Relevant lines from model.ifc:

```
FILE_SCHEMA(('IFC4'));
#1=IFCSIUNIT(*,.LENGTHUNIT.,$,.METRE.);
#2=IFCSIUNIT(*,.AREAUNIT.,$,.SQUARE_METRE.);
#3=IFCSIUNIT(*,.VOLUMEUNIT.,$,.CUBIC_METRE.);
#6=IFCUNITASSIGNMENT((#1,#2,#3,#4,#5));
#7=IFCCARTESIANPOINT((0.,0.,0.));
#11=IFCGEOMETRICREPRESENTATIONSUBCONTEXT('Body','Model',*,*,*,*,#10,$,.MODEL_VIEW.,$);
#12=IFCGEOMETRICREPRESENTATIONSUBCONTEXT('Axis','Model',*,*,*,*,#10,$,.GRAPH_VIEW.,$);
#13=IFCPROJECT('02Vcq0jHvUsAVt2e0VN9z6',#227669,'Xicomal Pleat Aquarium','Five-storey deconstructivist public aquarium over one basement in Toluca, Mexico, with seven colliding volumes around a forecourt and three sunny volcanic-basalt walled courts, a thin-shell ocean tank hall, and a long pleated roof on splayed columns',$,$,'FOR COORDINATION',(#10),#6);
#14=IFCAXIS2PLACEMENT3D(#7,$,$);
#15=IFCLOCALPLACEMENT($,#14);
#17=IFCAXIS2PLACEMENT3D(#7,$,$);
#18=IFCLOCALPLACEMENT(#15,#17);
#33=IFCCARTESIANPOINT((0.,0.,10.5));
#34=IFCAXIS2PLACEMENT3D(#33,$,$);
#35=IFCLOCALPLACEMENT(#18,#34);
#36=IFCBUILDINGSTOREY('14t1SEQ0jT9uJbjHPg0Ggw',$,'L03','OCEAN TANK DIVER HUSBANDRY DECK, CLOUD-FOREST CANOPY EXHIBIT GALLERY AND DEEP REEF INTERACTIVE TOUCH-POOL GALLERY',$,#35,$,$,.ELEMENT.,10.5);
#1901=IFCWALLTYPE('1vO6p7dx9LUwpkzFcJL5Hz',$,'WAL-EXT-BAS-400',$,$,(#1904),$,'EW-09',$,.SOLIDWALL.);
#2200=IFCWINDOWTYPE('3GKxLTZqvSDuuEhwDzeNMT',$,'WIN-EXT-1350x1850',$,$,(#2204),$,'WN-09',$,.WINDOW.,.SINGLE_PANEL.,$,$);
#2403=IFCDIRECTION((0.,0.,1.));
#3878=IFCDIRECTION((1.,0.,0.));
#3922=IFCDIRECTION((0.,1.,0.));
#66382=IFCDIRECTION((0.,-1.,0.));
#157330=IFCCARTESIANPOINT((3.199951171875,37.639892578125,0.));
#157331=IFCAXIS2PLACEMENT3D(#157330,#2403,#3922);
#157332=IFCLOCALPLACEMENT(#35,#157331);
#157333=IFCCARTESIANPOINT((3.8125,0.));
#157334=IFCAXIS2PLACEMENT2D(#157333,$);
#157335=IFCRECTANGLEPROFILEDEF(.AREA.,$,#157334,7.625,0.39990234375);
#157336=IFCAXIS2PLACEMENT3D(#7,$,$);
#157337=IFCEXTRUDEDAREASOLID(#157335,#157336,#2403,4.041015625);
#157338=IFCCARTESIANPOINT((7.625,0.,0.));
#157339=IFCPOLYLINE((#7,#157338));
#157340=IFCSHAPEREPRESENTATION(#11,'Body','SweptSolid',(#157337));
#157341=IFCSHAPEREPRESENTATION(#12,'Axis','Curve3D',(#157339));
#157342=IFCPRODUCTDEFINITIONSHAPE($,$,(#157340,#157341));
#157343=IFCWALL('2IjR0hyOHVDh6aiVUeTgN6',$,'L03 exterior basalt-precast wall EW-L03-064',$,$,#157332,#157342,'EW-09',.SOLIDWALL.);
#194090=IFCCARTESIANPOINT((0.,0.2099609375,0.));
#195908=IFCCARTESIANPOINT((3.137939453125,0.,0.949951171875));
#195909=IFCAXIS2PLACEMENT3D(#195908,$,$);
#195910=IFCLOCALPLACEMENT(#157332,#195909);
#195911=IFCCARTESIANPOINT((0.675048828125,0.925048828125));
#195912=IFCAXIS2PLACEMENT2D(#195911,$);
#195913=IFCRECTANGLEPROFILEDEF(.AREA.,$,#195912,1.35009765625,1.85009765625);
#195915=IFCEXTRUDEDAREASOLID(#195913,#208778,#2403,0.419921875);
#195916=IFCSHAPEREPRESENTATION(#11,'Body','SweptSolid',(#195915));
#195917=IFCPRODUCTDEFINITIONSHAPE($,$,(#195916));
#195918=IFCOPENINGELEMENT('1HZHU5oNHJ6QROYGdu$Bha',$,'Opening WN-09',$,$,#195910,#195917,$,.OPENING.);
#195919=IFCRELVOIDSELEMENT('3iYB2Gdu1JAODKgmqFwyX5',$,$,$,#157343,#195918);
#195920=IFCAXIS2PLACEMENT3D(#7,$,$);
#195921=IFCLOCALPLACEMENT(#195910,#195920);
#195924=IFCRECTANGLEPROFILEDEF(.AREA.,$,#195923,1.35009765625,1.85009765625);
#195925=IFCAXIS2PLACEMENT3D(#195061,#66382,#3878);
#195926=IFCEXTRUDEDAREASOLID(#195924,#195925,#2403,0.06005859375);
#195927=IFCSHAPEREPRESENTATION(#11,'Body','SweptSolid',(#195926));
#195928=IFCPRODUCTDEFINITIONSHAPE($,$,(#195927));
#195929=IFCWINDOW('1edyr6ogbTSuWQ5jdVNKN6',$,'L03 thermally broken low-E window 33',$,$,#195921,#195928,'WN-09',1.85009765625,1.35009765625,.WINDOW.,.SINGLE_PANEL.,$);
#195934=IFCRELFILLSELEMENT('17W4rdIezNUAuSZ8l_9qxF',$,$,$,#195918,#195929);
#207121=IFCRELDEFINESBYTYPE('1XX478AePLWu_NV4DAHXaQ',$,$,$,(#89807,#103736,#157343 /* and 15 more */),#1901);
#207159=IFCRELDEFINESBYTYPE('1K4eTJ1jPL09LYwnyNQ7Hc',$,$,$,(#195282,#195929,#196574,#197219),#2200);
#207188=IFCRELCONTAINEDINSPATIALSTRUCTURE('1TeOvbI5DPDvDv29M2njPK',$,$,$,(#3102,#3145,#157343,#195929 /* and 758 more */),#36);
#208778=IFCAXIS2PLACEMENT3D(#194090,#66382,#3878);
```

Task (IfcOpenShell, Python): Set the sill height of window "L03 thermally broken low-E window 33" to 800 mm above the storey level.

```python
import numpy as np
import ifcopenshell
import ifcopenshell.api.geometry
import ifcopenshell.geom
import ifcopenshell.util.element
import ifcopenshell.util.placement
import ifcopenshell.util.shape
import ifcopenshell.util.unit

model = ifcopenshell.open("model.ifc")
unit_scale = ifcopenshell.util.unit.calculate_unit_scale(model)

window = model.by_guid("1edyr6ogbTSuWQ5jdVNKN6")
opening = window.FillsVoids[0].RelatingOpeningElement
storey = ifcopenshell.util.element.get_container(window, ifc_class="IfcBuildingStorey")
level = ifcopenshell.util.placement.get_local_placement(storey.ObjectPlacement)[2, 3]

# The opening's origin need not be at the sill, so measure its lowest point.
shape = ifcopenshell.geom.create_shape(ifcopenshell.geom.settings(), opening)
bottom = ifcopenshell.util.shape.get_shape_bottom_elevation(shape, shape.geometry) / unit_scale
dz = level + 0.8 - bottom

shift = np.array([0.0, 0.0, dz])
# The window is placed relative to its opening, so it follows when the opening moves.
matrix = ifcopenshell.util.placement.get_local_placement(opening.ObjectPlacement)
matrix[:3, 3] += shift
ifcopenshell.api.geometry.edit_object_placement(
    model, product=opening, matrix=matrix, is_si=False, should_transform_children=True
)

print(f"moved by {dz * unit_scale:+.3f} m")

model.write("model_v2.ifc")
```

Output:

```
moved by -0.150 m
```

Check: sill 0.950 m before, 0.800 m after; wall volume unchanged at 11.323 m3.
